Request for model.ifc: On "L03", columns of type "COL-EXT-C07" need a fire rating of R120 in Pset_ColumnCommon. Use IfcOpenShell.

First a look at what the model holds.

```python
import ifcopenshell
import ifcopenshell.util.element

model = ifcopenshell.open("model.ifc")
print(model.schema)
storey = next(s for s in model.by_type("IfcBuildingStorey") if s.Name == "L03")
columns = [e for e in ifcopenshell.util.element.get_decomposition(storey) if e.is_a("IfcColumn")]
seen = {}
for e in columns:
    element_type = ifcopenshell.util.element.get_type(e)
    key = (element_type.Name if element_type != e and element_type else None, ifcopenshell.util.element.get_pset(e, "Pset_ColumnCommon", "FireRating"))
    seen[key] = seen.get(key, 0) + 1
for (name, value), count in sorted(seen.items(), key=str):
    print(count, "x", name, "|", value)
```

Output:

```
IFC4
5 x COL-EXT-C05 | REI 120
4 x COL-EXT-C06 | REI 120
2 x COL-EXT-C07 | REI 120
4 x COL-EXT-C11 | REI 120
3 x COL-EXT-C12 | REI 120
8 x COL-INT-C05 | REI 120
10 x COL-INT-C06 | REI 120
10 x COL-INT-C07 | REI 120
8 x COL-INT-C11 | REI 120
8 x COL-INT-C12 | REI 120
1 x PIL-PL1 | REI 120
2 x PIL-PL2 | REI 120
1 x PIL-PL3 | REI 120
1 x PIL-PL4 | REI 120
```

```python
import ifcopenshell
import ifcopenshell.api.pset
import ifcopenshell.util.element

model = ifcopenshell.open("model.ifc")

storey = next(s for s in model.by_type("IfcBuildingStorey") if s.Name == "L03")
columns = [e for e in ifcopenshell.util.element.get_decomposition(storey) if e.is_a("IfcColumn")]

count = 0
for e in columns:
    element_type = ifcopenshell.util.element.get_type(e)
    if element_type in (None, e) or element_type.Name != "COL-EXT-C07":
        continue
    # add_pset returns the element's existing set when there is one.
    pset = ifcopenshell.api.pset.add_pset(model, product=e, name="Pset_ColumnCommon")
    ifcopenshell.api.pset.edit_pset(model, pset=pset, properties={"FireRating": "R120"})
    count += 1

print(count, "columns updated")

model.write("model_edited.ifc")
```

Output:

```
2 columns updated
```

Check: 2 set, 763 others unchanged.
